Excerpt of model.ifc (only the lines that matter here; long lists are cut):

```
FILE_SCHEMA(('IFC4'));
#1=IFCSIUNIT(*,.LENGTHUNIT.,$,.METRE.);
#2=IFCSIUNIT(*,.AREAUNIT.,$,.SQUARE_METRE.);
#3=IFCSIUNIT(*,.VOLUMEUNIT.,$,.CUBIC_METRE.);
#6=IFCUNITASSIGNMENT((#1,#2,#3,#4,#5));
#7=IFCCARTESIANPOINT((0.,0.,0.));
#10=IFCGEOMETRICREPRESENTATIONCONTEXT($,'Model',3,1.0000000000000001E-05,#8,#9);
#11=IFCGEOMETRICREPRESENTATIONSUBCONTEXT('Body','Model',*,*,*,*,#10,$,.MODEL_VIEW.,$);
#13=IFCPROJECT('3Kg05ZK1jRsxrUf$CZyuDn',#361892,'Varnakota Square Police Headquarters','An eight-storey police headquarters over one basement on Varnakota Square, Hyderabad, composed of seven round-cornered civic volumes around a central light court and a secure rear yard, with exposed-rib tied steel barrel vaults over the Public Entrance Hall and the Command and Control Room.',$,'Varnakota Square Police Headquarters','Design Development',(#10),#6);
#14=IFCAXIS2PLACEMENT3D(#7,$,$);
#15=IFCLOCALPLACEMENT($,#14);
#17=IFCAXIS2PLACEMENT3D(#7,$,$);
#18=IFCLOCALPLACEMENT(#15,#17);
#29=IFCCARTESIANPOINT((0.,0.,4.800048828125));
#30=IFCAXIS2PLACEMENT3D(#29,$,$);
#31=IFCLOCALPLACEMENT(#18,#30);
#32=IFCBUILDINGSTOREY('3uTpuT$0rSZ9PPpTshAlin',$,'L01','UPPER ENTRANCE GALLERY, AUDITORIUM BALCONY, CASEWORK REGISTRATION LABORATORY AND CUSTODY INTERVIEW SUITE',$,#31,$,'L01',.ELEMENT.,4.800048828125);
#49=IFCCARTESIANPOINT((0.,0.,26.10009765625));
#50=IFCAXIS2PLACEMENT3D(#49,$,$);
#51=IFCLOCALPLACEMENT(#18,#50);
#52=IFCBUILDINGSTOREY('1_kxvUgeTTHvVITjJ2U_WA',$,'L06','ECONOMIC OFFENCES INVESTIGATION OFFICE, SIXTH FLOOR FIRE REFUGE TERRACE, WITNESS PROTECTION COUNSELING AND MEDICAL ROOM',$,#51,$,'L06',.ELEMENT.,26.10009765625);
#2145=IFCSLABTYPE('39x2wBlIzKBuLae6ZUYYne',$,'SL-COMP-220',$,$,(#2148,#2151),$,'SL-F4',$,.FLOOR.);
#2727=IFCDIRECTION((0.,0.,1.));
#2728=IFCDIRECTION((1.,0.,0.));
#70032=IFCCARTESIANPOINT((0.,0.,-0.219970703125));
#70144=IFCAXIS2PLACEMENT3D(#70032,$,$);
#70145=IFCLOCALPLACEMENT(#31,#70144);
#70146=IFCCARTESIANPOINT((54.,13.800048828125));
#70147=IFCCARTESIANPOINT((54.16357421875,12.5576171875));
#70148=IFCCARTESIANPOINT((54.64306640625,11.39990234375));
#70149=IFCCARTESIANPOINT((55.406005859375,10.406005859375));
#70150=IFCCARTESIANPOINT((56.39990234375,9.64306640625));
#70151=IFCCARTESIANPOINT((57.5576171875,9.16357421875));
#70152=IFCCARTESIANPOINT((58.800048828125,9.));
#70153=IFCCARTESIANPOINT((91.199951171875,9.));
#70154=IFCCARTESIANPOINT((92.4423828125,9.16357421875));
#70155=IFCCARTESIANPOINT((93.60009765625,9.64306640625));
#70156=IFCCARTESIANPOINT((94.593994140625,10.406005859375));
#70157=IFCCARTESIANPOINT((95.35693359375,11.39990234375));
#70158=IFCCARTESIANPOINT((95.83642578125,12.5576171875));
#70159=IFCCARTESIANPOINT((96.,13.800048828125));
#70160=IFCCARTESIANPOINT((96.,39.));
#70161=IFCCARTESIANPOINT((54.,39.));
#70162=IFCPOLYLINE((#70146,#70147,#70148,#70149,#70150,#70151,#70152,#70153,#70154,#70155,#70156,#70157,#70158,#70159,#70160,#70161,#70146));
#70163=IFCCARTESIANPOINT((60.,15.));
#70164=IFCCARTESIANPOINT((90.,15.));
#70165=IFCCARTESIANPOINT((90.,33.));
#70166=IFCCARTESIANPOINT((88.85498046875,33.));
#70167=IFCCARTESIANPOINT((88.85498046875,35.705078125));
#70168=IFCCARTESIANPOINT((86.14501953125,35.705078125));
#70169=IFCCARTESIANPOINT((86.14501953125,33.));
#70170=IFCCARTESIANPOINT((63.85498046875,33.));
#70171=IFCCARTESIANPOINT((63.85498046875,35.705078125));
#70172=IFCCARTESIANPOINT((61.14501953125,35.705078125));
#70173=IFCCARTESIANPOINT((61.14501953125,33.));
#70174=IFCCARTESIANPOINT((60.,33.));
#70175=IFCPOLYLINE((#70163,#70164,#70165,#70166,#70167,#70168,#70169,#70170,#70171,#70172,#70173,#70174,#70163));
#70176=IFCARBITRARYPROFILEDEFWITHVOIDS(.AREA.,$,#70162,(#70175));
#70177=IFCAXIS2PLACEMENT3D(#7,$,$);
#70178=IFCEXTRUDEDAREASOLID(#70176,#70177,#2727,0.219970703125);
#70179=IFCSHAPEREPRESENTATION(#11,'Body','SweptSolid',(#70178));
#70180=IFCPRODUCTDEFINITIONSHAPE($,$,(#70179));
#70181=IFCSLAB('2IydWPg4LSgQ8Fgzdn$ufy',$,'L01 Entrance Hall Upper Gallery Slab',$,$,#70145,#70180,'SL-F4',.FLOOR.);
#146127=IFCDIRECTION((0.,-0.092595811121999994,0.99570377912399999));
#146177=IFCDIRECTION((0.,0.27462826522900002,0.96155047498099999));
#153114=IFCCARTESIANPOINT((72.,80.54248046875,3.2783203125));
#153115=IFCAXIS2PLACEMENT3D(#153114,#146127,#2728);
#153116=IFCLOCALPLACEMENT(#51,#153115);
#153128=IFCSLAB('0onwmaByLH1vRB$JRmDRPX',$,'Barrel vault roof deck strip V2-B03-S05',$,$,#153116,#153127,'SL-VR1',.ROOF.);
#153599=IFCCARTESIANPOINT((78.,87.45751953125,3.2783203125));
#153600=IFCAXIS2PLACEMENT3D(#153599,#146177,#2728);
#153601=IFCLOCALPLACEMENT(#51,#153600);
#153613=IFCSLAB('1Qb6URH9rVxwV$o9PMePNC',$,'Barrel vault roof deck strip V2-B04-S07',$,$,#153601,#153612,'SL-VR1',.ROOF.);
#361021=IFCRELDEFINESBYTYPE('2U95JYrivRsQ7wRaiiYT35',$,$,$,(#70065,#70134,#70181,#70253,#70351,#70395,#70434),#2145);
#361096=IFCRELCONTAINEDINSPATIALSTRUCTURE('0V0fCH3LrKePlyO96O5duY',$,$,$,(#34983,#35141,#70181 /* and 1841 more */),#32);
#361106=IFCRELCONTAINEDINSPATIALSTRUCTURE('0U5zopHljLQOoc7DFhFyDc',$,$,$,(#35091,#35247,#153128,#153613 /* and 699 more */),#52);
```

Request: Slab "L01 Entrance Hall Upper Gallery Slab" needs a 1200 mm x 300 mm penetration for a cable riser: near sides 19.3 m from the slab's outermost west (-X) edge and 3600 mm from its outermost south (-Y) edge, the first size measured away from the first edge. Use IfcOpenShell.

```python
import numpy as np
import ifcopenshell
import ifcopenshell.api.feature
import ifcopenshell.api.geometry
import ifcopenshell.api.root
import ifcopenshell.geom
import ifcopenshell.util.placement
import ifcopenshell.util.representation
import ifcopenshell.util.shape
import ifcopenshell.util.unit

model = ifcopenshell.open("model.ifc")
unit_scale = ifcopenshell.util.unit.calculate_unit_scale(model)
settings = ifcopenshell.geom.settings()


def volume(element):
    """Net volume in cubic metres, openings subtracted."""
    shape = ifcopenshell.geom.create_shape(settings, element)
    return ifcopenshell.util.shape.get_volume(shape.geometry)


slab = model.by_guid("2IydWPg4LSgQ8Fgzdn$ufy")
before = volume(slab)

# Extent in the slab's own axes, in metres. The edges named are its -X and -Y sides.
slab_shape = ifcopenshell.geom.create_shape(settings, slab)
vertices = ifcopenshell.util.shape.get_vertices(slab_shape.geometry)
x_min, y_min, bottom = vertices.min(axis=0)
top = vertices[:, 2].max()

opening = ifcopenshell.api.root.create_entity(model, ifc_class="IfcOpeningElement", name="Cable riser opening", predefined_type="OPENING")
context = ifcopenshell.util.representation.get_context(model, "Model", "Body", "MODEL_VIEW")
width, depth = 1.2, 0.3
outline = [(0.0, 0.0), (width, 0.0), (width, depth), (0.0, depth), (0.0, 0.0)]
# Overshoot both faces by 50 mm so the cut is clean.
shape = ifcopenshell.api.geometry.add_slab_representation(
    model, context=context, depth=top - bottom + 0.1, polyline=outline
)
ifcopenshell.api.geometry.assign_representation(model, product=opening, representation=shape)

matrix = ifcopenshell.util.placement.get_local_placement(slab.ObjectPlacement)
matrix[:, 3] = matrix @ np.append(np.array([x_min + 19.3, y_min + 3.6, bottom - 0.05]) / unit_scale, 1.0)
ifcopenshell.api.geometry.edit_object_placement(model, product=opening, matrix=matrix, is_si=False)
ifcopenshell.api.feature.add_feature(model, feature=opening, element=slab)

after = volume(slab)

print(f"slab volume {before:.3f} -> {after:.3f} m3")

model.write("model_edited.ifc")
```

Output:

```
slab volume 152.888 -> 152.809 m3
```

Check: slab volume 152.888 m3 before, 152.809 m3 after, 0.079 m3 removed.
